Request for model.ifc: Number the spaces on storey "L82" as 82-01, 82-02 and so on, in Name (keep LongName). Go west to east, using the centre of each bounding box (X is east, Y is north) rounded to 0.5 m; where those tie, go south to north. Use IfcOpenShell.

First a look at what the model holds.

```python
import ifcopenshell
import ifcopenshell.util.element
import ifcopenshell.util.placement

model = ifcopenshell.open("model.ifc")
print(model.schema)
storey = next(s for s in model.by_type("IfcBuildingStorey") if s.Name == "L82")
spaces = [e for e in ifcopenshell.util.element.get_decomposition(storey) if e.is_a("IfcSpace")]
for e in sorted(spaces, key=lambda e: e.id()):
    origin = ifcopenshell.util.placement.get_local_placement(e.ObjectPlacement)[:3, 3]
    print(e.id(), e.Name, e.LongName, origin.round(2) + 0.0, sep=" | ")
```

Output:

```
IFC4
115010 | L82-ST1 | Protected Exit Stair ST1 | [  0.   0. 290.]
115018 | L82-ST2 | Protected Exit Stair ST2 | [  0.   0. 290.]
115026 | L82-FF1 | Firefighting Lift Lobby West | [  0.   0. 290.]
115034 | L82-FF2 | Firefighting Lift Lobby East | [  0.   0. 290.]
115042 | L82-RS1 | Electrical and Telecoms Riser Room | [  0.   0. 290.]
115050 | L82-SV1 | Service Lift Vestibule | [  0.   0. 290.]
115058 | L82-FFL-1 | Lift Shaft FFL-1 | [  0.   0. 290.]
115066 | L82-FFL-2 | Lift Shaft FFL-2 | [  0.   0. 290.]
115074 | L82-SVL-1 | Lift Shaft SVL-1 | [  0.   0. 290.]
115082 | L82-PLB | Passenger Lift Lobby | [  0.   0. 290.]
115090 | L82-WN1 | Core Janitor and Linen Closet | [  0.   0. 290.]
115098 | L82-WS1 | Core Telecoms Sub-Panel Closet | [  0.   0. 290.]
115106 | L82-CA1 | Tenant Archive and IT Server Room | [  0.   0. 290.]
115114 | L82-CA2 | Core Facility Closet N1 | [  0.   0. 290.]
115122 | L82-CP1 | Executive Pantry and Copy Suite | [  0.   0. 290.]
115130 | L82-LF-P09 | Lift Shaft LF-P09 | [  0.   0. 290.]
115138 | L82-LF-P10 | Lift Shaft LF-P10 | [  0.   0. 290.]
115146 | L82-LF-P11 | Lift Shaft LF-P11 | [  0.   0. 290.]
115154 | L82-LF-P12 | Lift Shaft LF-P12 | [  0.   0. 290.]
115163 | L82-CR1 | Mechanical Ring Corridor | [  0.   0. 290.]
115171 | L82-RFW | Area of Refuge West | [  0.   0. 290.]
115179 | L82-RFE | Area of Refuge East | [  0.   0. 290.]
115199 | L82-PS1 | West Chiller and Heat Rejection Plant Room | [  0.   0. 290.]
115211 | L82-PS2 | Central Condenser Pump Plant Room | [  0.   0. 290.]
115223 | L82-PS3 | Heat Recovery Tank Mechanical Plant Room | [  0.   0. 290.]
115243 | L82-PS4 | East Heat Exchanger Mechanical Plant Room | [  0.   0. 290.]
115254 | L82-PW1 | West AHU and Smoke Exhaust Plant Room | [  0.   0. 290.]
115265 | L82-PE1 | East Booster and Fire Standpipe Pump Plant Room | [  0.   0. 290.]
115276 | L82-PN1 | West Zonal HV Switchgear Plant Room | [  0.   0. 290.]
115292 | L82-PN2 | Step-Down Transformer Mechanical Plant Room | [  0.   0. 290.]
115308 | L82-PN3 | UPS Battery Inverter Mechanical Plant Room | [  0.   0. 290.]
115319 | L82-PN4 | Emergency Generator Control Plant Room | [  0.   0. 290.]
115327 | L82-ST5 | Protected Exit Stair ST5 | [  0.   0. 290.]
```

```python
import ifcopenshell
import ifcopenshell.geom
import ifcopenshell.util.element
import ifcopenshell.util.shape

model = ifcopenshell.open("model.ifc")
settings = ifcopenshell.geom.settings()
settings.set("use-world-coords", True)


def centre(element):
    shape = ifcopenshell.geom.create_shape(settings, element)
    return ifcopenshell.util.shape.get_bbox_centroid(shape.geometry)


storey = next(s for s in model.by_type("IfcBuildingStorey") if s.Name == "L82")
spaces = [e for e in ifcopenshell.util.element.get_decomposition(storey) if e.is_a("IfcSpace")]

# Insertion points can sit at a corner or the storey origin, so sort by the geometry (in metres).
centres = {e: centre(e) for e in spaces}
spaces.sort(key=lambda e: (round(centres[e][0] / 0.5), centres[e][1]))

for i, e in enumerate(spaces, start=1):
    number = f"82-{i:02d}"
    e.Name = number
    print(e.id(), number)

model.write("model_rev.ifc")
```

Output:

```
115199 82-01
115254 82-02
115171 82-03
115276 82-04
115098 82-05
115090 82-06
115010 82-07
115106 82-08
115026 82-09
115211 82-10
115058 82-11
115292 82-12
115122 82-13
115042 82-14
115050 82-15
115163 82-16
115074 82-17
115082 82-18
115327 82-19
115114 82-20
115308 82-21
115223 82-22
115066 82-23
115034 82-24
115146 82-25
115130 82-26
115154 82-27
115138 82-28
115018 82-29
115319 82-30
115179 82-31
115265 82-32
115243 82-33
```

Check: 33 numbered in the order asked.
